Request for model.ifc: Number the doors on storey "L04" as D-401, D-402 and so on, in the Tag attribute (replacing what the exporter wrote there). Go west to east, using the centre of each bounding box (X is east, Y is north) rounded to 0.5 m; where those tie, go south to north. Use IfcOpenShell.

First a look at what the model holds.

```python
import ifcopenshell
import ifcopenshell.util.element
import ifcopenshell.util.placement

model = ifcopenshell.open("model.ifc")
print(model.schema)
storey = next(s for s in model.by_type("IfcBuildingStorey") if s.Name == "L04")
doors = [e for e in ifcopenshell.util.element.get_decomposition(storey) if e.is_a("IfcDoor")]
for e in sorted(doors, key=lambda e: e.id()):
    origin = ifcopenshell.util.placement.get_local_placement(e.ObjectPlacement)[:3, 3]
    print(e.id(), e.Tag, e.Name, origin.round(2) + 0.0, sep=" | ")
```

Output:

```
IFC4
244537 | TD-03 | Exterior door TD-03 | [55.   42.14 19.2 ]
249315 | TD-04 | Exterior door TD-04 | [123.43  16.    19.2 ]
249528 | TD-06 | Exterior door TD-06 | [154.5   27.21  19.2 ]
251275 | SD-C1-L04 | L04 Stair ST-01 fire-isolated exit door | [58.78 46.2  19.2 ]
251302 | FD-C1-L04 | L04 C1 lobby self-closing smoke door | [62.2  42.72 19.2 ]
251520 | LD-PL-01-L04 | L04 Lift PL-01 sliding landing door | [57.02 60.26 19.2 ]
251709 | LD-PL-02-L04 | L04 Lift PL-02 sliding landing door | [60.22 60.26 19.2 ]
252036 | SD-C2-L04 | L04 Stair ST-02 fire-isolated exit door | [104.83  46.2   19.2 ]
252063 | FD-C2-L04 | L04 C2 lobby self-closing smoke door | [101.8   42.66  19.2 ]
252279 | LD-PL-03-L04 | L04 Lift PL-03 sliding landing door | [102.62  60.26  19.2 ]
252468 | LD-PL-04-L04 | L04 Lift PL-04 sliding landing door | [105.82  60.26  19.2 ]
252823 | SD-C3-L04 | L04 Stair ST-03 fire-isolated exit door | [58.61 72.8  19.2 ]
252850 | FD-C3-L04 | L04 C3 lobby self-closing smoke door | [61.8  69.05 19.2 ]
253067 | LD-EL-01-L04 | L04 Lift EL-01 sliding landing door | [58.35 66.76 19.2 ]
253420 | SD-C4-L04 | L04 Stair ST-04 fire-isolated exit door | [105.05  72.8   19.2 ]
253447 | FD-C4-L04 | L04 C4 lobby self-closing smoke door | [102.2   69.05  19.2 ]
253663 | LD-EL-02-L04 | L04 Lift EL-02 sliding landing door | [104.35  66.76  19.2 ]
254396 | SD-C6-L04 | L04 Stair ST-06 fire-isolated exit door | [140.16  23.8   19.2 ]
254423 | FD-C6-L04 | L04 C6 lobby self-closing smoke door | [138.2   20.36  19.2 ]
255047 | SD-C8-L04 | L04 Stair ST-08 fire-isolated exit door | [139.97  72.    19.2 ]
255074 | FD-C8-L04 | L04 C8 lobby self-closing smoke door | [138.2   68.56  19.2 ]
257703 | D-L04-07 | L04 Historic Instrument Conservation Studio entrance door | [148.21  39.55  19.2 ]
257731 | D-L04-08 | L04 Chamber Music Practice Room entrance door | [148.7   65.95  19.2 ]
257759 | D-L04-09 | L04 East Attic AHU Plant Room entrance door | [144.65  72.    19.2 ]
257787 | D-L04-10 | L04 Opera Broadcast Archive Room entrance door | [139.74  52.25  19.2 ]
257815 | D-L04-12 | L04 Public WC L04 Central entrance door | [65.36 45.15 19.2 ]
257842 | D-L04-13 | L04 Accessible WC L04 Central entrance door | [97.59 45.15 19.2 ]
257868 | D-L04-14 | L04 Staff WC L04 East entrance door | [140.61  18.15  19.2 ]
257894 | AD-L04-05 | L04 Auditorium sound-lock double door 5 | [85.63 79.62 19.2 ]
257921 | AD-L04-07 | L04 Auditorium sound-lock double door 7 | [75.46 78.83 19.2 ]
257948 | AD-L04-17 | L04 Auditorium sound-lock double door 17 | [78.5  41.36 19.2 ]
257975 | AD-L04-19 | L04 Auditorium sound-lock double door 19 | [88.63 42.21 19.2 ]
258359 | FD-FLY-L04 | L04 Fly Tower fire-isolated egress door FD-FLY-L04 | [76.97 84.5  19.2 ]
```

```python
import ifcopenshell
import ifcopenshell.geom
import ifcopenshell.util.element
import ifcopenshell.util.shape

model = ifcopenshell.open("model.ifc")
settings = ifcopenshell.geom.settings()
settings.set("use-world-coords", True)


def centre(element):
    shape = ifcopenshell.geom.create_shape(settings, element)
    return ifcopenshell.util.shape.get_bbox_centroid(shape.geometry)


storey = next(s for s in model.by_type("IfcBuildingStorey") if s.Name == "L04")
doors = [e for e in ifcopenshell.util.element.get_decomposition(storey) if e.is_a("IfcDoor")]

# Insertion points can sit at a corner or the storey origin, so sort by the geometry (in metres).
centres = {e: centre(e) for e in doors}
doors.sort(key=lambda e: (round(centres[e][0] / 0.5), centres[e][1]))

for i, e in enumerate(doors, start=1):
    number = f"D-4{i:02d}"
    e.Tag = number
    print(e.id(), number)

model.write("model_edited.ifc")
```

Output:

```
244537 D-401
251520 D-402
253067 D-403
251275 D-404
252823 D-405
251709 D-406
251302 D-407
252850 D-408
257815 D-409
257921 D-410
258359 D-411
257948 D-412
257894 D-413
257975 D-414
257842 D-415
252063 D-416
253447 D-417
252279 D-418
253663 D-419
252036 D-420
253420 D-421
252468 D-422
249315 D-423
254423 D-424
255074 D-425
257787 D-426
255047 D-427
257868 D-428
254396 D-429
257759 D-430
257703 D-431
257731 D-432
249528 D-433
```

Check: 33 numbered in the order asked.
